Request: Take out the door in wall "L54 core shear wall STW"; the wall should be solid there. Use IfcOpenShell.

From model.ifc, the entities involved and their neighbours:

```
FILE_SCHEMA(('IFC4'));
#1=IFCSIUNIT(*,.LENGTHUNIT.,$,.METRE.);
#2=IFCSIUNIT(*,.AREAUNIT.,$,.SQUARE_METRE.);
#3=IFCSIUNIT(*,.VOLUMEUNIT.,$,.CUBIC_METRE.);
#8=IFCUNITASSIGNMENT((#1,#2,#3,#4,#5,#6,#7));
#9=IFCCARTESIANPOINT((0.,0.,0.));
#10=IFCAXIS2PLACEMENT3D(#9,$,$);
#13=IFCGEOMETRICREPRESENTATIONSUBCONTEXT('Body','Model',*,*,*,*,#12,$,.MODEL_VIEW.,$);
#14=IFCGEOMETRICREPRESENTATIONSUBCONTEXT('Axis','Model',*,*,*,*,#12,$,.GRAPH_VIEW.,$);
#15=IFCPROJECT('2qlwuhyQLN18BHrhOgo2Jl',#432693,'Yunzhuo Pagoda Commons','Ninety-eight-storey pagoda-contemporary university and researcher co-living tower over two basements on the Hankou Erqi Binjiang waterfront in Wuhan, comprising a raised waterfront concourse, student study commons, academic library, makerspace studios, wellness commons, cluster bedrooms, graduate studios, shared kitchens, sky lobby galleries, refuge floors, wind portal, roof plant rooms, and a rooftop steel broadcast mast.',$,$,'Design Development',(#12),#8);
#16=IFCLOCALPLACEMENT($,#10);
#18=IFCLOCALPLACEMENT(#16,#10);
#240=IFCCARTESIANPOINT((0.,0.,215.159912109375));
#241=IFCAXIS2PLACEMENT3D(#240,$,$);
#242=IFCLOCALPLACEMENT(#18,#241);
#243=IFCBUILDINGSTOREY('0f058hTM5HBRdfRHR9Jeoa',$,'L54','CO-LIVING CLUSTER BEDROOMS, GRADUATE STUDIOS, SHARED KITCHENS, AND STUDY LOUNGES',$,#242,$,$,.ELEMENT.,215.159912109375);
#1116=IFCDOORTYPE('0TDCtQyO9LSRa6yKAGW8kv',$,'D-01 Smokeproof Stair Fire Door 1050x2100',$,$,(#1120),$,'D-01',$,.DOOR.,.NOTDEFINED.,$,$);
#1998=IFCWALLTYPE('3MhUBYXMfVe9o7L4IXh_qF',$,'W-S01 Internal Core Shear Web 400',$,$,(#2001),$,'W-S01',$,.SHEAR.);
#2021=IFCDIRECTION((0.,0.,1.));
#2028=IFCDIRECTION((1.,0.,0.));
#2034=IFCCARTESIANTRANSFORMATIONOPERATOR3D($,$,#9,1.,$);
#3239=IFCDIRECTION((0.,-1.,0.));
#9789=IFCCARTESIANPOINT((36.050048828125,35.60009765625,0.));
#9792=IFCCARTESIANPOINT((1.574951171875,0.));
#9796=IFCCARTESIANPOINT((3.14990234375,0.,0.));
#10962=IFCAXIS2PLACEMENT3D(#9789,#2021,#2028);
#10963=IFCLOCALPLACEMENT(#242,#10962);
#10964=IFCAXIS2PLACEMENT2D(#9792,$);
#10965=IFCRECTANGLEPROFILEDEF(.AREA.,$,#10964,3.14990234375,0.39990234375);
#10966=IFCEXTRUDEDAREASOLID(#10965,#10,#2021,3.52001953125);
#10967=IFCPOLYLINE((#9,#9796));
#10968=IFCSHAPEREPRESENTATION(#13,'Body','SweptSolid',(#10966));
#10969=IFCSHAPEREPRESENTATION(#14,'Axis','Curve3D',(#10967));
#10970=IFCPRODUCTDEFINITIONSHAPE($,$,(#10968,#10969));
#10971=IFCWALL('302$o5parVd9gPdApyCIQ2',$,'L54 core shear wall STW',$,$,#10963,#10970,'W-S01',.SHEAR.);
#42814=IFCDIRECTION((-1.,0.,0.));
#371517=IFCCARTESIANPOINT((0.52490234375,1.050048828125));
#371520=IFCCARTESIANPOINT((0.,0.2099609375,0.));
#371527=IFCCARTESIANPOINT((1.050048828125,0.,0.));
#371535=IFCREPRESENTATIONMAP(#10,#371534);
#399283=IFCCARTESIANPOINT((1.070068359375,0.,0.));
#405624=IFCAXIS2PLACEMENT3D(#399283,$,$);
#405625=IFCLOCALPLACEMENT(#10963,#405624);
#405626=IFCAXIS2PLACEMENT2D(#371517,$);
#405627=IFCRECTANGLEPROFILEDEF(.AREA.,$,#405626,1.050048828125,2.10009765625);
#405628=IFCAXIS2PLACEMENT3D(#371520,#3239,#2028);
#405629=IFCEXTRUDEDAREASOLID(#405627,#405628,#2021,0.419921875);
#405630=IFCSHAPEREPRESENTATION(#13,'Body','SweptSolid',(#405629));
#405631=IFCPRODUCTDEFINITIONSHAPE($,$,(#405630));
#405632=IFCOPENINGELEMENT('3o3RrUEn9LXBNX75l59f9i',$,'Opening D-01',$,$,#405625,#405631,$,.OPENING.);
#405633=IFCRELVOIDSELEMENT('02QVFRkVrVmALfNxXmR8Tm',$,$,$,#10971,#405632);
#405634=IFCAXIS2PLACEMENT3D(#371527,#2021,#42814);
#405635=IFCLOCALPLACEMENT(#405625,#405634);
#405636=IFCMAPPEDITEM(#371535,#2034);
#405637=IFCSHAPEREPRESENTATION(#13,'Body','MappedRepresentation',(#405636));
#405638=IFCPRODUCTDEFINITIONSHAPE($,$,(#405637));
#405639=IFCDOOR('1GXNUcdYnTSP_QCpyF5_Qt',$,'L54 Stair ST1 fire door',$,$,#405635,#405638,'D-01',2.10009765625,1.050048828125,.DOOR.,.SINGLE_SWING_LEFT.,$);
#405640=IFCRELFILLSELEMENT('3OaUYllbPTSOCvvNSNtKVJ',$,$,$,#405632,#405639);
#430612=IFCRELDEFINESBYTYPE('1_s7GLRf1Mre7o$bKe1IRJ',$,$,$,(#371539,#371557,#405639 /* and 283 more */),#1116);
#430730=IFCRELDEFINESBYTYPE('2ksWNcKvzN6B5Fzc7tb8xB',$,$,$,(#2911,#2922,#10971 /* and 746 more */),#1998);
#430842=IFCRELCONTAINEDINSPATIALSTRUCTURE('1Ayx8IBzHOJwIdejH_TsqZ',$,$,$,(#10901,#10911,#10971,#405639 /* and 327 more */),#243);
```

```python
import ifcopenshell
import ifcopenshell.api.feature
import ifcopenshell.api.root
import ifcopenshell.geom
import ifcopenshell.util.shape

model = ifcopenshell.open("model.ifc")
settings = ifcopenshell.geom.settings()


def volume(element):
    """Net volume in cubic metres, openings subtracted."""
    shape = ifcopenshell.geom.create_shape(settings, element)
    return ifcopenshell.util.shape.get_volume(shape.geometry)


door = model.by_guid("1GXNUcdYnTSP_QCpyF5_Qt")
opening = door.FillsVoids[0].RelatingOpeningElement
wall = opening.VoidsElements[0].RelatingBuildingElement
before = volume(wall)

ifcopenshell.api.root.remove_product(model, product=door)
ifcopenshell.api.feature.remove_feature(model, feature=opening)

after = volume(wall)

print(f"wall volume {before:.3f} -> {after:.3f} m3")

model.write("model_rev.ifc")
```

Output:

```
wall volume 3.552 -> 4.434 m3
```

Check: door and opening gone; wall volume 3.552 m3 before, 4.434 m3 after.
